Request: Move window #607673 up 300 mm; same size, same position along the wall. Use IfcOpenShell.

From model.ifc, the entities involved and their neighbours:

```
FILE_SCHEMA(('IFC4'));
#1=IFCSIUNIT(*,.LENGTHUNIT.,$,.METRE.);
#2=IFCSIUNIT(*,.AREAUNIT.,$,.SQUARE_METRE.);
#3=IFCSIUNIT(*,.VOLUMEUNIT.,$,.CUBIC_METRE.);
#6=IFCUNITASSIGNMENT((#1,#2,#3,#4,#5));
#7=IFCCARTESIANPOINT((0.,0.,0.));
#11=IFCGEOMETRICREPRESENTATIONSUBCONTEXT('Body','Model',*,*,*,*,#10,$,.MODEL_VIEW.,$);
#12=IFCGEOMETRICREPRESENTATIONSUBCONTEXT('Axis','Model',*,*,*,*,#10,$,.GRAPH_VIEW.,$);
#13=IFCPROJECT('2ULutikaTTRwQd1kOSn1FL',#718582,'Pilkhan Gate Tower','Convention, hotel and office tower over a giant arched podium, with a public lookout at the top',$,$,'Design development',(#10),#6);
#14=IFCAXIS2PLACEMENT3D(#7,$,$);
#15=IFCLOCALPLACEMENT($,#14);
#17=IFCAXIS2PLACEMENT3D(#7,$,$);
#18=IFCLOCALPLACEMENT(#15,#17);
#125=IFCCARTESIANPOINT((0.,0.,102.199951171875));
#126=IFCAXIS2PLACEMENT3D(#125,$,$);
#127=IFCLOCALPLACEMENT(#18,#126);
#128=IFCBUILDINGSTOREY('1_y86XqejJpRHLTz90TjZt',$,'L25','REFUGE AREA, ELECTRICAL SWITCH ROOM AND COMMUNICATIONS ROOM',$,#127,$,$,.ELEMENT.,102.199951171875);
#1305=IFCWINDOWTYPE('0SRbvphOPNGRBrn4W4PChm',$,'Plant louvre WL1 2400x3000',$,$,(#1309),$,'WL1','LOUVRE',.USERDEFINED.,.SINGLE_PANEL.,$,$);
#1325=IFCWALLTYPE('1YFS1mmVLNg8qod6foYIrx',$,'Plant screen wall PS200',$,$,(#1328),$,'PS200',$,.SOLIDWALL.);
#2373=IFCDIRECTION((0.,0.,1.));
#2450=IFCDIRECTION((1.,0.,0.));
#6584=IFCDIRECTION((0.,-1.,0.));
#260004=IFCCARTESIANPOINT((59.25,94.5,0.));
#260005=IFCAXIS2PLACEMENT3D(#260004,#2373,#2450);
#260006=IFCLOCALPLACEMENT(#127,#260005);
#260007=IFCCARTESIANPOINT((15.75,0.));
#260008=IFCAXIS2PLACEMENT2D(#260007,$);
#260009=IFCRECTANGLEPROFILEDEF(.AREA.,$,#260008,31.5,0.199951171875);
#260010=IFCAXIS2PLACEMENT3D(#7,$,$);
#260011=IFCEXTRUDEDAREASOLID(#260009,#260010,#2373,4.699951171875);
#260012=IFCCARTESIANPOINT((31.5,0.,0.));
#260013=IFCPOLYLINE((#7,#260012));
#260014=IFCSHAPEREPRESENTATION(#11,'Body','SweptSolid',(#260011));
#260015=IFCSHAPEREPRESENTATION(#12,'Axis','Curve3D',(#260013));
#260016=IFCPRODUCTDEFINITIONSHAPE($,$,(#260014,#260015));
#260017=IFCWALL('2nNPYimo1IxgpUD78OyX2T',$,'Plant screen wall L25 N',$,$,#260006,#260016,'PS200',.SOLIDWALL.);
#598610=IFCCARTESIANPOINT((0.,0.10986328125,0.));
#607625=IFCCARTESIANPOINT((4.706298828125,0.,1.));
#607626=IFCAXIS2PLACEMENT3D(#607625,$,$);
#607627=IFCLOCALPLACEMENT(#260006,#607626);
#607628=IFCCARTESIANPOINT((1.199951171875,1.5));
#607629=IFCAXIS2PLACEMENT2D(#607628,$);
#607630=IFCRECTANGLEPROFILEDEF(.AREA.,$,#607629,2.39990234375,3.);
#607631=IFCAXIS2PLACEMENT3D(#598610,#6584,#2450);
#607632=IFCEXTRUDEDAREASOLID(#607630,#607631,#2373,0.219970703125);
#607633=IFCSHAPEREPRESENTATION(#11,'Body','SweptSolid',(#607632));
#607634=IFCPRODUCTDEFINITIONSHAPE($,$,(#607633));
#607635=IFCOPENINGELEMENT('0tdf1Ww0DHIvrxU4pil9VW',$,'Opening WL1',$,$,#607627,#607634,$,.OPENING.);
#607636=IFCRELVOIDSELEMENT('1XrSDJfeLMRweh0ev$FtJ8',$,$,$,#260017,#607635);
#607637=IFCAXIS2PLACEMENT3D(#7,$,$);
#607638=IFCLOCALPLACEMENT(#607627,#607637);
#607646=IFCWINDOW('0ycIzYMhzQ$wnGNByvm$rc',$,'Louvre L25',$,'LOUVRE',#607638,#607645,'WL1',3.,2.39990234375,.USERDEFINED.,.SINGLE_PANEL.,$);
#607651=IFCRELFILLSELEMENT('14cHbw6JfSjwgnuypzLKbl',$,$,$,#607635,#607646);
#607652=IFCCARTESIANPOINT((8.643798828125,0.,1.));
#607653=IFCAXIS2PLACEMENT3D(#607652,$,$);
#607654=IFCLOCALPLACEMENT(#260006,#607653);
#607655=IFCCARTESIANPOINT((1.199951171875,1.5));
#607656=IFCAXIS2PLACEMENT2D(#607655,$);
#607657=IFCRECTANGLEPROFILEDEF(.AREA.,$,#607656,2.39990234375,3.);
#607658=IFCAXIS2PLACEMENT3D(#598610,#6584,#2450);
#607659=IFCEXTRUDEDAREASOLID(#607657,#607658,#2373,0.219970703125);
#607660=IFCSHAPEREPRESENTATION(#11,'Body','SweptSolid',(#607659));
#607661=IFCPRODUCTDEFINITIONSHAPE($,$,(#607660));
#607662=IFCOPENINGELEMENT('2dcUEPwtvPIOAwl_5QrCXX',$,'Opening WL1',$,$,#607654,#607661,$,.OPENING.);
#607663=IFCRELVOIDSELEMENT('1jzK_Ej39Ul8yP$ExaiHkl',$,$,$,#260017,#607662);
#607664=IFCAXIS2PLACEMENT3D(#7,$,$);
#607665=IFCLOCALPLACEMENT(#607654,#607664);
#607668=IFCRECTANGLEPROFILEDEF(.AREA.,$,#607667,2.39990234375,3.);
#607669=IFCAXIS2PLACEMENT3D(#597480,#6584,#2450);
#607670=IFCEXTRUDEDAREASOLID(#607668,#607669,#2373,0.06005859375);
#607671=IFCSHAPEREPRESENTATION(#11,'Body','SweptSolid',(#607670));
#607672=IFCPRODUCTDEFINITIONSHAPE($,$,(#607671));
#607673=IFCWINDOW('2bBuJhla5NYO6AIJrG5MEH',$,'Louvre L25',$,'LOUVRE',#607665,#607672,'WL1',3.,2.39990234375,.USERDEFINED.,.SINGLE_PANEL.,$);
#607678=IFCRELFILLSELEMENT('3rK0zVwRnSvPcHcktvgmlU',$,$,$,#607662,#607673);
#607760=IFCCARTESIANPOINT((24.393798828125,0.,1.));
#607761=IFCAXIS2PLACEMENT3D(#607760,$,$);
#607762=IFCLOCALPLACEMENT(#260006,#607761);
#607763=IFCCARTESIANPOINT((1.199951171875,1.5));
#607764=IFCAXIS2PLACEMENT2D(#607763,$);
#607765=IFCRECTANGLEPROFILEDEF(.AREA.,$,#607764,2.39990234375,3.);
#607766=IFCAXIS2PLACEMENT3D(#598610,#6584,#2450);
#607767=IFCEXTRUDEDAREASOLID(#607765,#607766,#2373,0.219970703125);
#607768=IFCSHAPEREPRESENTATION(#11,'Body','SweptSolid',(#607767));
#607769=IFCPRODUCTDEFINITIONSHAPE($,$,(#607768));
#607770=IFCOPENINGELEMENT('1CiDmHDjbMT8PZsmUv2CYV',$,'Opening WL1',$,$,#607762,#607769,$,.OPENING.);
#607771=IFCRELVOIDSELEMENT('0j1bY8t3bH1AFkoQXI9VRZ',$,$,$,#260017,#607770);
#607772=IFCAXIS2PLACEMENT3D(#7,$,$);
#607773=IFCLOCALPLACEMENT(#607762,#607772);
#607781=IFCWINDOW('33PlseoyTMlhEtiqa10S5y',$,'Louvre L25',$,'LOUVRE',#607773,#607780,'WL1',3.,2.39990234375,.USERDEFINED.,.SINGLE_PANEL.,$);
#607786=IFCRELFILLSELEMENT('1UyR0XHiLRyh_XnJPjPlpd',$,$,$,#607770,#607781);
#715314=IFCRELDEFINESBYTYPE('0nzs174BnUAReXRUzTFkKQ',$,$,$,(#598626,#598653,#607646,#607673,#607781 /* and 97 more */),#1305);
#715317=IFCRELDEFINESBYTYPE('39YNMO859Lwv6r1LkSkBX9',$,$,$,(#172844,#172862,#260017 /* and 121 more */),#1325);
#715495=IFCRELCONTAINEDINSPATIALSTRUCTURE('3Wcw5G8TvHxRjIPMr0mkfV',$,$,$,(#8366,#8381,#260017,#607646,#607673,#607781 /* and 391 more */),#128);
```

```python
import numpy as np
import ifcopenshell
import ifcopenshell.api.geometry
import ifcopenshell.util.placement
import ifcopenshell.util.unit

model = ifcopenshell.open("model.ifc")
unit_scale = ifcopenshell.util.unit.calculate_unit_scale(model)

window = model.by_id(607673)
opening = window.FillsVoids[0].RelatingOpeningElement
dz = 0.3

shift = np.array([0.0, 0.0, dz])
# The window is placed relative to its opening, so it follows when the opening moves.
matrix = ifcopenshell.util.placement.get_local_placement(opening.ObjectPlacement)
matrix[:3, 3] += shift
ifcopenshell.api.geometry.edit_object_placement(
    model, product=opening, matrix=matrix, is_si=False, should_transform_children=True
)

print(f"moved by {dz * unit_scale:+.3f} m")

model.write("model_edited.ifc")
```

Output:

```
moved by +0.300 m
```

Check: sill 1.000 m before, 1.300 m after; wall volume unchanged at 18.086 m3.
